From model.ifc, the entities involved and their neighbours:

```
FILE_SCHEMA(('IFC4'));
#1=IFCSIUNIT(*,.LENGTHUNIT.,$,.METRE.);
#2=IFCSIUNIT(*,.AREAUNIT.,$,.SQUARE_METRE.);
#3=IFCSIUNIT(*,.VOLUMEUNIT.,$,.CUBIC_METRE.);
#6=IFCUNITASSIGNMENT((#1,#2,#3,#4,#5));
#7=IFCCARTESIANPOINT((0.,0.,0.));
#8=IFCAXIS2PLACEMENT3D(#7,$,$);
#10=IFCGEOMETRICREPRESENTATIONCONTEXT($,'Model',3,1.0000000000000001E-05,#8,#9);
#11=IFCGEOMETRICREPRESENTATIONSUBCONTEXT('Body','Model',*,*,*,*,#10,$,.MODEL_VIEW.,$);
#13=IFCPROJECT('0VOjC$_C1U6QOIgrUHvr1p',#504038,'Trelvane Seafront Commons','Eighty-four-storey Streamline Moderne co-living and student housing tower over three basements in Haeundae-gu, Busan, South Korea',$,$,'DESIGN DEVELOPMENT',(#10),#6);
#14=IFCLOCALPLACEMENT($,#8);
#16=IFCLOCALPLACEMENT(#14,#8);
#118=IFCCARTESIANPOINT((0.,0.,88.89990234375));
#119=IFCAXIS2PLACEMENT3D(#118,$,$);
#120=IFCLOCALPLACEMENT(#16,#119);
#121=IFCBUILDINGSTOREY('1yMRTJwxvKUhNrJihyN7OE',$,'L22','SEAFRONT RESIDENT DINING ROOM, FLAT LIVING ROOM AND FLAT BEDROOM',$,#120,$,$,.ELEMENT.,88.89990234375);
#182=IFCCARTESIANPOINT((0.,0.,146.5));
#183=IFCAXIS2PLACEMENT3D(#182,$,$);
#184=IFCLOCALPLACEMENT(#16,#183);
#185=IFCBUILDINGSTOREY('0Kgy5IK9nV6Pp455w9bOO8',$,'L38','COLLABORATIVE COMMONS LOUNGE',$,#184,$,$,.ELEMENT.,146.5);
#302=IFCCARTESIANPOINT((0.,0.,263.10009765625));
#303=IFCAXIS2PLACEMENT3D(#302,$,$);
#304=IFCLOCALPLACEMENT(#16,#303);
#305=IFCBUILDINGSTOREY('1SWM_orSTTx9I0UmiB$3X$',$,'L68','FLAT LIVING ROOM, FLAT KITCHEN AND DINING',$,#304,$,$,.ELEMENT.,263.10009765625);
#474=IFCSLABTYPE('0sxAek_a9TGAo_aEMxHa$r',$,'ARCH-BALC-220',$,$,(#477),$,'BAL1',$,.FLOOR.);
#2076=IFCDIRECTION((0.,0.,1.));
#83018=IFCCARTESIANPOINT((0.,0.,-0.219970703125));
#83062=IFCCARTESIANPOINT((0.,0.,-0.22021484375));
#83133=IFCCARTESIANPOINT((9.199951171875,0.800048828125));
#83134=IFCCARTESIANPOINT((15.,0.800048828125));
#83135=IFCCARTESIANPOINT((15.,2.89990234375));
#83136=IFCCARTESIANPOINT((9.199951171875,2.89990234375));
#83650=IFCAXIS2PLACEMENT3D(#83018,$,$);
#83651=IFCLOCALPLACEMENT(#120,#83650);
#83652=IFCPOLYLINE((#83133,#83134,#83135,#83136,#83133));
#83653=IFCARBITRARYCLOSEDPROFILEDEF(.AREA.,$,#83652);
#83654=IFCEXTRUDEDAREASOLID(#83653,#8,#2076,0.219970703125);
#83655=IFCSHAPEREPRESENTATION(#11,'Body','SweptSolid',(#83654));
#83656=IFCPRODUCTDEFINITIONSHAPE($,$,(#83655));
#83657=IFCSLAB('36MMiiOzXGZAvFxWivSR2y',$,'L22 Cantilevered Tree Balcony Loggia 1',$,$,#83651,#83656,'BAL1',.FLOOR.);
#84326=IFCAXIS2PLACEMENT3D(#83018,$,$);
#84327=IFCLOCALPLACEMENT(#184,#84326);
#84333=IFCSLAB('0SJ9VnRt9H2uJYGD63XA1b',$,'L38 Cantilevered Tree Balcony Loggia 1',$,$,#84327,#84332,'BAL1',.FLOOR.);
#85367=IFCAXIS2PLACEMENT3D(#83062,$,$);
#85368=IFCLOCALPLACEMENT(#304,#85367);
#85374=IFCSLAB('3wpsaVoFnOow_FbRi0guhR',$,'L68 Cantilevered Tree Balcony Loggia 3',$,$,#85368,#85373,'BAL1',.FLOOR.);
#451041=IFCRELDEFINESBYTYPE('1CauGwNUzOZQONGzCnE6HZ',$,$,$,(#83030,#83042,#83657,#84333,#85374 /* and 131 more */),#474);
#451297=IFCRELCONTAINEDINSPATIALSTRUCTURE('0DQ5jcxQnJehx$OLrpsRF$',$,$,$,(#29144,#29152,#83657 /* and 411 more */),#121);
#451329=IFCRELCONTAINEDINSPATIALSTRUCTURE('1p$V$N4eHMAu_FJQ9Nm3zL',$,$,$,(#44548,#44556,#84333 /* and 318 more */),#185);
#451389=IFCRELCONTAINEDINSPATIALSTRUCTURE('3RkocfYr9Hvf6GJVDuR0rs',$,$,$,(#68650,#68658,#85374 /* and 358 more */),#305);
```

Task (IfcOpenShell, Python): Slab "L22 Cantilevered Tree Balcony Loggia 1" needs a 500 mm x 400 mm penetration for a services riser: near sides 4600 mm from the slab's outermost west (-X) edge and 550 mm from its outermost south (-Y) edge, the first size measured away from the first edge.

```python
import numpy as np
import ifcopenshell
import ifcopenshell.api.feature
import ifcopenshell.api.geometry
import ifcopenshell.api.root
import ifcopenshell.geom
import ifcopenshell.util.placement
import ifcopenshell.util.representation
import ifcopenshell.util.shape
import ifcopenshell.util.unit

model = ifcopenshell.open("model.ifc")
unit_scale = ifcopenshell.util.unit.calculate_unit_scale(model)
settings = ifcopenshell.geom.settings()


def volume(element):
    """Net volume in cubic metres, openings subtracted."""
    shape = ifcopenshell.geom.create_shape(settings, element)
    return ifcopenshell.util.shape.get_volume(shape.geometry)


slab = model.by_id(83657)
before = volume(slab)

# Extent in the slab's own axes, in metres. The edges named are its -X and -Y sides.
slab_shape = ifcopenshell.geom.create_shape(settings, slab)
vertices = ifcopenshell.util.shape.get_vertices(slab_shape.geometry)
x_min, y_min, bottom = vertices.min(axis=0)
top = vertices[:, 2].max()

opening = ifcopenshell.api.root.create_entity(model, ifc_class="IfcOpeningElement", name="Services riser opening", predefined_type="OPENING")
context = ifcopenshell.util.representation.get_context(model, "Model", "Body", "MODEL_VIEW")
width, depth = 0.5, 0.4
outline = [(0.0, 0.0), (width, 0.0), (width, depth), (0.0, depth), (0.0, 0.0)]
# Overshoot both faces by 50 mm so the cut is clean.
shape = ifcopenshell.api.geometry.add_slab_representation(
    model, context=context, depth=top - bottom + 0.1, polyline=outline
)
ifcopenshell.api.geometry.assign_representation(model, product=opening, representation=shape)

matrix = ifcopenshell.util.placement.get_local_placement(slab.ObjectPlacement)
matrix[:, 3] = matrix @ np.append(np.array([x_min + 4.6, y_min + 0.55, bottom - 0.05]) / unit_scale, 1.0)
ifcopenshell.api.geometry.edit_object_placement(model, product=opening, matrix=matrix, is_si=False)
ifcopenshell.api.feature.add_feature(model, feature=opening, element=slab)

after = volume(slab)

print(f"slab volume {before:.3f} -> {after:.3f} m3")

model.write("model_rev.ifc")
```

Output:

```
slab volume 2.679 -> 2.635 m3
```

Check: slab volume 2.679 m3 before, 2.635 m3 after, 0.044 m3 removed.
